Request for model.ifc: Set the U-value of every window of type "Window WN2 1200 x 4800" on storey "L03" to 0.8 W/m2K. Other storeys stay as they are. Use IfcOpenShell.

First a look at what the model holds.

```python
import ifcopenshell
import ifcopenshell.util.element

model = ifcopenshell.open("model.ifc")
print(model.schema)
storey = next(s for s in model.by_type("IfcBuildingStorey") if s.Name == "L03")
windows = [e for e in ifcopenshell.util.element.get_decomposition(storey) if e.is_a("IfcWindow")]
seen = {}
for e in windows:
    element_type = ifcopenshell.util.element.get_type(e)
    key = (element_type.Name if element_type != e and element_type else None, ifcopenshell.util.element.get_pset(e, "Pset_WindowCommon", "ThermalTransmittance"))
    seen[key] = seen.get(key, 0) + 1
for (name, value), count in sorted(seen.items(), key=str):
    print(count, "x", name, "|", value)
```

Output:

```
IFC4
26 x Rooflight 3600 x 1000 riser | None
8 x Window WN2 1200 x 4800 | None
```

```python
import ifcopenshell
import ifcopenshell.api.pset
import ifcopenshell.util.element

model = ifcopenshell.open("model.ifc")

storey = next(s for s in model.by_type("IfcBuildingStorey") if s.Name == "L03")
windows = [e for e in ifcopenshell.util.element.get_decomposition(storey) if e.is_a("IfcWindow")]

count = 0
for e in windows:
    element_type = ifcopenshell.util.element.get_type(e)
    if element_type in (None, e) or element_type.Name != "Window WN2 1200 x 4800":
        continue
    # add_pset returns the element's existing set when there is one.
    pset = ifcopenshell.api.pset.add_pset(model, product=e, name="Pset_WindowCommon")
    ifcopenshell.api.pset.edit_pset(model, pset=pset, properties={"ThermalTransmittance": 0.8})
    count += 1

print(count, "windows updated")

model.write("model-out.ifc")
```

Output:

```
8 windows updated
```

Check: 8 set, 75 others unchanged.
